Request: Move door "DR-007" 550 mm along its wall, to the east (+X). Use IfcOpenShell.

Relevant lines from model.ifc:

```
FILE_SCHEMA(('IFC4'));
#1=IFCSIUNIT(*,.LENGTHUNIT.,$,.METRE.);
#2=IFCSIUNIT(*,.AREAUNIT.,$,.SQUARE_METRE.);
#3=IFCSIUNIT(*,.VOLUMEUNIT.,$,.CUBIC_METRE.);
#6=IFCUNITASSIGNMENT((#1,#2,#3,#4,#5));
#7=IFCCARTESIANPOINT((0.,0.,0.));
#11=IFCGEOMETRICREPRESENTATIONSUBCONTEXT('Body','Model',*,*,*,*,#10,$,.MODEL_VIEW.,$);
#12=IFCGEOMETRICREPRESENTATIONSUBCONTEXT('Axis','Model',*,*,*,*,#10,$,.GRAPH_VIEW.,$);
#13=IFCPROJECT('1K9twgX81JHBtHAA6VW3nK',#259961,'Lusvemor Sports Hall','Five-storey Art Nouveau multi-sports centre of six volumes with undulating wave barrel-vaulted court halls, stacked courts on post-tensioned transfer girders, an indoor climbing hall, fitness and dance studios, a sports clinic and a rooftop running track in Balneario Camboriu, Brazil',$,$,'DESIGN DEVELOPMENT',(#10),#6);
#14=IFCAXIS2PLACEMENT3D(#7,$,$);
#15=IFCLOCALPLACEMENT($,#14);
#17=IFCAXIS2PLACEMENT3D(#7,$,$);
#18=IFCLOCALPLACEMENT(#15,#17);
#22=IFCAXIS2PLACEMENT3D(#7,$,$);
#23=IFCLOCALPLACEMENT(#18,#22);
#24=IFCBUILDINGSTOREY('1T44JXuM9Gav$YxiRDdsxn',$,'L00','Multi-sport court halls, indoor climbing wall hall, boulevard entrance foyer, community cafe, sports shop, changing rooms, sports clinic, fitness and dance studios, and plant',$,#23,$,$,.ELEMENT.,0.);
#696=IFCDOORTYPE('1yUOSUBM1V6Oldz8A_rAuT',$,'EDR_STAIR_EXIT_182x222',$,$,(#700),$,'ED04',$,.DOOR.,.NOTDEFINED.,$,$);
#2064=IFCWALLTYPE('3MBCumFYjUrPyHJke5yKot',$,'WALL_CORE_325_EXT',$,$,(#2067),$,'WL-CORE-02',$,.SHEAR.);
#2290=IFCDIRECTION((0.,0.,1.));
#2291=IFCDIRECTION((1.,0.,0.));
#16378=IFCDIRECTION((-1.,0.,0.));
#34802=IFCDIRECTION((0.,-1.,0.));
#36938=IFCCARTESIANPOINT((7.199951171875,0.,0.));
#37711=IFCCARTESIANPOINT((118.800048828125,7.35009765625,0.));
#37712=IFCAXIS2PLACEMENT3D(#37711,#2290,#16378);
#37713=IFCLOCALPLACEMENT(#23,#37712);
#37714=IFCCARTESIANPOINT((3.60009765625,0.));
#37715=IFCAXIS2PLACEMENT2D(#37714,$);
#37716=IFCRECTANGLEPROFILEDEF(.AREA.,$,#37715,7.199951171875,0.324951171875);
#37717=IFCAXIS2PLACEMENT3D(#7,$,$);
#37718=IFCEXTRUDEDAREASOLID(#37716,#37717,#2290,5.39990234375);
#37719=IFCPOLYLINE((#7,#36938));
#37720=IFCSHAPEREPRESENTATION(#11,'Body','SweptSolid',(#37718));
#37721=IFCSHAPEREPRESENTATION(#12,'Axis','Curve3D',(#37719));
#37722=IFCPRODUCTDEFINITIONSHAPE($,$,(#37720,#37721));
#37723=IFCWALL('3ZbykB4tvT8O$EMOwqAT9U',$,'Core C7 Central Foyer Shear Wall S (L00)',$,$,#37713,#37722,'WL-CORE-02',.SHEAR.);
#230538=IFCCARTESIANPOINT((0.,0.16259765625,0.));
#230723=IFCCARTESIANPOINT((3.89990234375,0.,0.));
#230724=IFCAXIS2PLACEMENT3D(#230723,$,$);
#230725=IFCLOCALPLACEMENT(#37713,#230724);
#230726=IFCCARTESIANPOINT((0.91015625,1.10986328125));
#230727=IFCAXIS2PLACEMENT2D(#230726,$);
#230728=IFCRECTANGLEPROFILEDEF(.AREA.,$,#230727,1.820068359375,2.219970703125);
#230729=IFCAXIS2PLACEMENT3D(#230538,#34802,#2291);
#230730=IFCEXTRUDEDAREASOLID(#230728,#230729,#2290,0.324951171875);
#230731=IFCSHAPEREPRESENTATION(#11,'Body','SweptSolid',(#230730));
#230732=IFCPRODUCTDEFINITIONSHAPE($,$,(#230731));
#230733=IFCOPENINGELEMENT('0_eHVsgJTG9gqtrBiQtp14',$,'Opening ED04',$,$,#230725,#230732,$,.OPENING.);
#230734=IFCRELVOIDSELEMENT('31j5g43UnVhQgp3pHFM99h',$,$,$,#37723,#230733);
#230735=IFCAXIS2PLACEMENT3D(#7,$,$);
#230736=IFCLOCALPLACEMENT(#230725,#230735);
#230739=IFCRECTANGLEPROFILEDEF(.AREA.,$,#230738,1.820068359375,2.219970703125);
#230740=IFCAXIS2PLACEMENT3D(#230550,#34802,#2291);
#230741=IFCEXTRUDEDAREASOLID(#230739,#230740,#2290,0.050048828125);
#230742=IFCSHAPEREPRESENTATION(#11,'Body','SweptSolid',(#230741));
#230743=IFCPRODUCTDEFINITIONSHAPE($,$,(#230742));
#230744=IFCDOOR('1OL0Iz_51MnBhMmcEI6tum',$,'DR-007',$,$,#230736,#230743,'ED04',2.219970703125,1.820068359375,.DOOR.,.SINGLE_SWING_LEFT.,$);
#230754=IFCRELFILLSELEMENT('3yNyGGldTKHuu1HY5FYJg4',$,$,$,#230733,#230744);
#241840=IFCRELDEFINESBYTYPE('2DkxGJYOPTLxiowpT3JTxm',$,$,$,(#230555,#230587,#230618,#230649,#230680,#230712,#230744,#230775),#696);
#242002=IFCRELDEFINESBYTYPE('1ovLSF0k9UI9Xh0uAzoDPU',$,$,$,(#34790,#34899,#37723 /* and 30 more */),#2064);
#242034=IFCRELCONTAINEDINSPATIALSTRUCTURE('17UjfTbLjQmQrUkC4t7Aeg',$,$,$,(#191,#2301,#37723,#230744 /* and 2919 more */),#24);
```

```python
import ifcopenshell
import ifcopenshell.api.geometry
import ifcopenshell.util.placement
import ifcopenshell.util.unit

model = ifcopenshell.open("model.ifc")
unit_scale = ifcopenshell.util.unit.calculate_unit_scale(model)

door = model.by_id(230744)
opening = door.FillsVoids[0].RelatingOpeningElement
wall = opening.VoidsElements[0].RelatingBuildingElement

wall_matrix = ifcopenshell.util.placement.get_local_placement(wall.ObjectPlacement)
shift = wall_matrix[:3, 0] * -0.55 / unit_scale
before = ifcopenshell.util.placement.get_local_placement(door.ObjectPlacement)[:3, 3].copy()

# The door is placed relative to its opening, so it follows when the opening moves.
matrix = ifcopenshell.util.placement.get_local_placement(opening.ObjectPlacement)
matrix[:3, 3] += shift
ifcopenshell.api.geometry.edit_object_placement(
    model, product=opening, matrix=matrix, is_si=False, should_transform_children=True
)

after = ifcopenshell.util.placement.get_local_placement(door.ObjectPlacement)[:3, 3]
print("door moved by", (after - before).round(3) + 0.0)

model.write("model-out.ifc")
```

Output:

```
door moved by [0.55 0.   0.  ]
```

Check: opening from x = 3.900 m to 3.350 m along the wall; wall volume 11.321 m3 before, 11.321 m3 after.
